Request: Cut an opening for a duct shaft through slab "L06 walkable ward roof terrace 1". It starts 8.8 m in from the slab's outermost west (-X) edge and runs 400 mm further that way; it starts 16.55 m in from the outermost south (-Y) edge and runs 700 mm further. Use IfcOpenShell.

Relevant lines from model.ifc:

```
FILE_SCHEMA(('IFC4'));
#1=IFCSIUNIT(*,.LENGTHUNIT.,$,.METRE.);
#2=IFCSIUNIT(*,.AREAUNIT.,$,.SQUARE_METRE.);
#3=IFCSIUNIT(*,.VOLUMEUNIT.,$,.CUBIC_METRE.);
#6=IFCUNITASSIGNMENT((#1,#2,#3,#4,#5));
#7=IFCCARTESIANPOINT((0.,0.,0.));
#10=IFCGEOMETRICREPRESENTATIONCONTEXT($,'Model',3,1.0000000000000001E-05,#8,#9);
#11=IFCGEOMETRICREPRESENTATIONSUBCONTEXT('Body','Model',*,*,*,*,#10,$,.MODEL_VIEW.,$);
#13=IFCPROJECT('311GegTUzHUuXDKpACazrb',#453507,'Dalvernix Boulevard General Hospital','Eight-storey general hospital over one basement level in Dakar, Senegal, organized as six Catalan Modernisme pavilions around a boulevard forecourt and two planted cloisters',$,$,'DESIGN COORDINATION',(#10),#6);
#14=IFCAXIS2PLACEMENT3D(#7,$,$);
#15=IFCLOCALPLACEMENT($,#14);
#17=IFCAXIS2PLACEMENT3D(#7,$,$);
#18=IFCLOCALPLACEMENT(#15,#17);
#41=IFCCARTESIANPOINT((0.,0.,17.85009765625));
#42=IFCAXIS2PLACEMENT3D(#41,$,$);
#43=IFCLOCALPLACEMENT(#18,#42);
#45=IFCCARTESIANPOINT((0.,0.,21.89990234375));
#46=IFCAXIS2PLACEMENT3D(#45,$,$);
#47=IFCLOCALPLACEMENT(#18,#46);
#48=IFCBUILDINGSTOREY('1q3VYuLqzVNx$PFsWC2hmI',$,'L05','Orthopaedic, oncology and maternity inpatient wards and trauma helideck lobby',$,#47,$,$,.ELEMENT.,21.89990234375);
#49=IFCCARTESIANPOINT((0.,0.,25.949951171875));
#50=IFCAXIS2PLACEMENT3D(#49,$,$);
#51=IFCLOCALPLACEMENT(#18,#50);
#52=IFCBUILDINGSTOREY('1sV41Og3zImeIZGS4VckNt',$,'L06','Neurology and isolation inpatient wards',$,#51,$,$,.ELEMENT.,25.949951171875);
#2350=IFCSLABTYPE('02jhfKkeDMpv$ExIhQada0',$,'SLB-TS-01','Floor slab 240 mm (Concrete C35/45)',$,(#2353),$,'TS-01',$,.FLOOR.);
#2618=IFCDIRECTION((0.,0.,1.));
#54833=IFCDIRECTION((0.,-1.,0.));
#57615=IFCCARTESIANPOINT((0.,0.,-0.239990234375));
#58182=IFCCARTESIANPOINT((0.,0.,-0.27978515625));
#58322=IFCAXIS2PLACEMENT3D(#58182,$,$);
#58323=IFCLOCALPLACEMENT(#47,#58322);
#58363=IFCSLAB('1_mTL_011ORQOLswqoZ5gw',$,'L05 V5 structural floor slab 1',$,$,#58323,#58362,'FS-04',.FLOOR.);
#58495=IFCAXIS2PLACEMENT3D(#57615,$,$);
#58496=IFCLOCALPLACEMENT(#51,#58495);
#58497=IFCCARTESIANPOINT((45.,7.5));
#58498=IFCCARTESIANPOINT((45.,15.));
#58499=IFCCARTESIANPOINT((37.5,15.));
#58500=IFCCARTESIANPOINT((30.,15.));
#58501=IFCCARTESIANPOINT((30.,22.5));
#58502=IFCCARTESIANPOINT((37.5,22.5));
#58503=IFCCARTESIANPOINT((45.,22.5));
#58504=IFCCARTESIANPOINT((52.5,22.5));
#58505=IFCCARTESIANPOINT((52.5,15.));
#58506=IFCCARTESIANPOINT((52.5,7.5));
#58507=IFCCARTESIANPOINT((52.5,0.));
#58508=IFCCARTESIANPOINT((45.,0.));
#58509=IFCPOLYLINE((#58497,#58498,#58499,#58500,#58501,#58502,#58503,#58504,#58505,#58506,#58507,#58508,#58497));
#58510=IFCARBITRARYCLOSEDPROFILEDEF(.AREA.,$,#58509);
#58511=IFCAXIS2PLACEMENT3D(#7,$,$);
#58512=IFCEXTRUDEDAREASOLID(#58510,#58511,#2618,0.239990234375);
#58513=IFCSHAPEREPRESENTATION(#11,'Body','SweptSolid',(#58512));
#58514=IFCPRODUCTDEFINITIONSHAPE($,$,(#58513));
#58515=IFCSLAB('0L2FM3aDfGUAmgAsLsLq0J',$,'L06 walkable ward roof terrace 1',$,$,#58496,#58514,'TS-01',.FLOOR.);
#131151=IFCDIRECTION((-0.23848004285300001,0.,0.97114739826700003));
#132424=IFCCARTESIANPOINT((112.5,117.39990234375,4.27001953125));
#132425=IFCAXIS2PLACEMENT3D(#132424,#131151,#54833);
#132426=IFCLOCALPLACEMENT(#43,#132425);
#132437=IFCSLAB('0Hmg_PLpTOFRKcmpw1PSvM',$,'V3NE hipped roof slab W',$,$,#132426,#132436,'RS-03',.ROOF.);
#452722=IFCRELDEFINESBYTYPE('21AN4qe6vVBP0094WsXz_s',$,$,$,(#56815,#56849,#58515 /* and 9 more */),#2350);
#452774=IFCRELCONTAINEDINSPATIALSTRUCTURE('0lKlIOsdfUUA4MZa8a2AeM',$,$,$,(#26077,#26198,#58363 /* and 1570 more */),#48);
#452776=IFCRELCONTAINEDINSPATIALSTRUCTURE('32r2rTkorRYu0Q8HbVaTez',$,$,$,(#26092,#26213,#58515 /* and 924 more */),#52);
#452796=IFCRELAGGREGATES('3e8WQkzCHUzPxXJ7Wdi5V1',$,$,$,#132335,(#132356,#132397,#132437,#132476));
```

```python
import numpy as np
import ifcopenshell
import ifcopenshell.api.feature
import ifcopenshell.api.geometry
import ifcopenshell.api.root
import ifcopenshell.geom
import ifcopenshell.util.placement
import ifcopenshell.util.representation
import ifcopenshell.util.shape
import ifcopenshell.util.unit

model = ifcopenshell.open("model.ifc")
unit_scale = ifcopenshell.util.unit.calculate_unit_scale(model)
settings = ifcopenshell.geom.settings()


def volume(element):
    """Net volume in cubic metres, openings subtracted."""
    shape = ifcopenshell.geom.create_shape(settings, element)
    return ifcopenshell.util.shape.get_volume(shape.geometry)


slab = model.by_guid("0L2FM3aDfGUAmgAsLsLq0J")
before = volume(slab)

# Extent in the slab's own axes, in metres. The edges named are its -X and -Y sides.
slab_shape = ifcopenshell.geom.create_shape(settings, slab)
vertices = ifcopenshell.util.shape.get_vertices(slab_shape.geometry)
x_min, y_min, bottom = vertices.min(axis=0)
top = vertices[:, 2].max()

opening = ifcopenshell.api.root.create_entity(model, ifc_class="IfcOpeningElement", name="Duct shaft opening", predefined_type="OPENING")
context = ifcopenshell.util.representation.get_context(model, "Model", "Body", "MODEL_VIEW")
width, depth = 0.4, 0.7
outline = [(0.0, 0.0), (width, 0.0), (width, depth), (0.0, depth), (0.0, 0.0)]
# Overshoot both faces by 50 mm so the cut is clean.
shape = ifcopenshell.api.geometry.add_slab_representation(
    model, context=context, depth=top - bottom + 0.1, polyline=outline
)
ifcopenshell.api.geometry.assign_representation(model, product=opening, representation=shape)

matrix = ifcopenshell.util.placement.get_local_placement(slab.ObjectPlacement)
matrix[:, 3] = matrix @ np.append(np.array([x_min + 8.8, y_min + 16.55, bottom - 0.05]) / unit_scale, 1.0)
ifcopenshell.api.geometry.edit_object_placement(model, product=opening, matrix=matrix, is_si=False)
ifcopenshell.api.feature.add_feature(model, feature=opening, element=slab)

after = volume(slab)

print(f"slab volume {before:.3f} -> {after:.3f} m3")

model.write("model_updated.ifc")
```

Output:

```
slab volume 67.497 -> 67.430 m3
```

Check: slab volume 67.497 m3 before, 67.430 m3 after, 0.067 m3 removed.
